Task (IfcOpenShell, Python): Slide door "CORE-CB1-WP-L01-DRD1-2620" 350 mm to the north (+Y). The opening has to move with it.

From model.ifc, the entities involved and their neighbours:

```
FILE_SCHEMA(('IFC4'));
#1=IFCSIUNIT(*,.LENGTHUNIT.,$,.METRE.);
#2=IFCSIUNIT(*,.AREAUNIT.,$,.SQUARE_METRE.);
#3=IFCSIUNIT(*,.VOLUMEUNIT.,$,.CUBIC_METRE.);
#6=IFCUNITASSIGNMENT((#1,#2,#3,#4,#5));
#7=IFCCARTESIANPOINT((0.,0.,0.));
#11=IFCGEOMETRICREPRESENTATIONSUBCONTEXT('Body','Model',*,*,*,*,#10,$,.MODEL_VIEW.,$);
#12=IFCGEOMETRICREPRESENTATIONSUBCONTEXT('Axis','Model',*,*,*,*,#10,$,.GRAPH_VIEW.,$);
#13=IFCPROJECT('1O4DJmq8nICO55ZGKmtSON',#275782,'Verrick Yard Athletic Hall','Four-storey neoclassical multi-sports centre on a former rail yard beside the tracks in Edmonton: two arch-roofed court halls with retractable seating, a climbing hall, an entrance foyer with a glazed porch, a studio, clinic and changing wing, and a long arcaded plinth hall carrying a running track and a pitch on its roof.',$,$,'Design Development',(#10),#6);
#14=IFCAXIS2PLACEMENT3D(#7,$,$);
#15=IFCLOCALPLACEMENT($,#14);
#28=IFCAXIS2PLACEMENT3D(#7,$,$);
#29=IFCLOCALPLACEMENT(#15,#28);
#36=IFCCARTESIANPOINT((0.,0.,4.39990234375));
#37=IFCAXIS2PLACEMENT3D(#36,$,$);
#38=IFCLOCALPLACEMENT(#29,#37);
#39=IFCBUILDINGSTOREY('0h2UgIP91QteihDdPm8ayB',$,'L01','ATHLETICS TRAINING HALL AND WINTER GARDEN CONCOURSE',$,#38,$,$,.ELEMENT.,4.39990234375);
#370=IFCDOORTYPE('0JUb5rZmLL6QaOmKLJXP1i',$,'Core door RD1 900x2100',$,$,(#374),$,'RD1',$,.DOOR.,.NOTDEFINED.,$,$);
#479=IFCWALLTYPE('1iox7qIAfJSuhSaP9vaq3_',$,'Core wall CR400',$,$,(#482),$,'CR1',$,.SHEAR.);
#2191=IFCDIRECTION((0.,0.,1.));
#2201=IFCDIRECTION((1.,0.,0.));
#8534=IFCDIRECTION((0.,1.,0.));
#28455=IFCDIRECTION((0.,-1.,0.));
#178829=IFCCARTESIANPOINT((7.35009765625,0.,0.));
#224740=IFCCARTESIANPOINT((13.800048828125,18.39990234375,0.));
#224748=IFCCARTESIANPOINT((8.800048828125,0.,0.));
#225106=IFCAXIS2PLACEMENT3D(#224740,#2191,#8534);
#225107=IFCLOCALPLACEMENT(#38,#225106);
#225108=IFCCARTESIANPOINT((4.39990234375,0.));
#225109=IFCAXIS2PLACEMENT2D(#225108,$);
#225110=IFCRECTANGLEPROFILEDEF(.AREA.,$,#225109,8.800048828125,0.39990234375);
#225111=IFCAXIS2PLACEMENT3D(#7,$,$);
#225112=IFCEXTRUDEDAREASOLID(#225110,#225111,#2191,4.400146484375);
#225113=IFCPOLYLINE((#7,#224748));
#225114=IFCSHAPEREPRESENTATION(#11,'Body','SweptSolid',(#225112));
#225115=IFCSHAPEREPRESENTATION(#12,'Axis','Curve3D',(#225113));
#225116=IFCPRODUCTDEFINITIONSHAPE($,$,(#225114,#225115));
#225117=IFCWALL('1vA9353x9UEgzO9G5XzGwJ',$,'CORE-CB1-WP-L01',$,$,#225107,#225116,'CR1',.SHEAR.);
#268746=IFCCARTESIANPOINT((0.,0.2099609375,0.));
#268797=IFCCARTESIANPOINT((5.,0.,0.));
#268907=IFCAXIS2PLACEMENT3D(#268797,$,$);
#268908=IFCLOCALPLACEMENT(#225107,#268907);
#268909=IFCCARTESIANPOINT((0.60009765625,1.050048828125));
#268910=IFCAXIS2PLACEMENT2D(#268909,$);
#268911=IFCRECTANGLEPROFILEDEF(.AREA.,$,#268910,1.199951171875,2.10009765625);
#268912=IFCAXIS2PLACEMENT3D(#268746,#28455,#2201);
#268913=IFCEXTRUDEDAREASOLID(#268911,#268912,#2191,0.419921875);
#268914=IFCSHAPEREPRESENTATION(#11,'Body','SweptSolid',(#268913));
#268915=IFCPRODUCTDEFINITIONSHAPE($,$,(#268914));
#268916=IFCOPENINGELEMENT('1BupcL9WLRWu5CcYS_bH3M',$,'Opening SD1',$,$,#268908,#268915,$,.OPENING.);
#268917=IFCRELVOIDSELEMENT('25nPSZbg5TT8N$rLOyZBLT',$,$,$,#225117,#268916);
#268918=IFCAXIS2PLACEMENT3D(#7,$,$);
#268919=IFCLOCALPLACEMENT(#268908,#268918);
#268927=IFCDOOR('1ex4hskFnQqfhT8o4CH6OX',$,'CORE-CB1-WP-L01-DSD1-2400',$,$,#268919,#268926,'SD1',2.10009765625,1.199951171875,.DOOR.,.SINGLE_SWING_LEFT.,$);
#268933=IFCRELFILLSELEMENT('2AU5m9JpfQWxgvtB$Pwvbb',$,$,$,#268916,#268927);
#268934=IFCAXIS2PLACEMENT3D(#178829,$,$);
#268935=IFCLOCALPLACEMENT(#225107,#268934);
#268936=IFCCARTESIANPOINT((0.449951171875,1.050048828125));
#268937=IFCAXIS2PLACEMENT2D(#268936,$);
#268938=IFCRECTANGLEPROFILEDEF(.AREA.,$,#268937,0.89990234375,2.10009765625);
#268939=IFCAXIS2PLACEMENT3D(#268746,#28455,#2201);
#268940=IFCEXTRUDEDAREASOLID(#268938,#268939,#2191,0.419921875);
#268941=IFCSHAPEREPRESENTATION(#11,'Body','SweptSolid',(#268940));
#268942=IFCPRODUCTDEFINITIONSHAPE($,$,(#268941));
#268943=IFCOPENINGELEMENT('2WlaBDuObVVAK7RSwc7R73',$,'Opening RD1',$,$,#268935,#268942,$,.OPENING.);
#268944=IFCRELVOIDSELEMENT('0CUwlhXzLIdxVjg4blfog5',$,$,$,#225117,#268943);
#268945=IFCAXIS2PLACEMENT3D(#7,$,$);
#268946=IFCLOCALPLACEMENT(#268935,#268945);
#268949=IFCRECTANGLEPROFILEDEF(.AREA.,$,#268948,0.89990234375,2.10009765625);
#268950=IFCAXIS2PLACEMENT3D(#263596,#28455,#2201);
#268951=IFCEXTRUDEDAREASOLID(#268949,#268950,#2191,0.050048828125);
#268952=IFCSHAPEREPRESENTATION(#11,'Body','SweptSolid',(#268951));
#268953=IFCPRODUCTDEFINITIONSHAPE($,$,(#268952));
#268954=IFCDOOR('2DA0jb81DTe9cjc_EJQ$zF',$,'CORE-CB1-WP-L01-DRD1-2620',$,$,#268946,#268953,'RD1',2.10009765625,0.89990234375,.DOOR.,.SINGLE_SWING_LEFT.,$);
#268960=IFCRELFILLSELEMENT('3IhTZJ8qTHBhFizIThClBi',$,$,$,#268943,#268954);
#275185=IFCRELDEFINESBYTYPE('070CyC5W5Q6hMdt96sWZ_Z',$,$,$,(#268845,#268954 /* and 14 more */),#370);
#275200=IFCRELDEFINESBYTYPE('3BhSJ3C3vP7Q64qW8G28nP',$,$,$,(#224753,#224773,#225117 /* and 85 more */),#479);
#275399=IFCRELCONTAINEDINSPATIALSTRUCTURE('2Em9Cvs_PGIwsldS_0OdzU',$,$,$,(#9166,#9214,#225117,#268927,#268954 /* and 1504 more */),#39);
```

```python
import ifcopenshell
import ifcopenshell.api.geometry
import ifcopenshell.util.placement

model = ifcopenshell.open("model.ifc")

door = model.by_guid("2DA0jb81DTe9cjc_EJQ$zF")
opening = door.FillsVoids[0].RelatingOpeningElement
wall = opening.VoidsElements[0].RelatingBuildingElement

wall_matrix = ifcopenshell.util.placement.get_local_placement(wall.ObjectPlacement)
shift = wall_matrix[:3, 0] * 0.35
before = ifcopenshell.util.placement.get_local_placement(door.ObjectPlacement)[:3, 3].copy()

# The door is placed relative to its opening, so it follows when the opening moves.
matrix = ifcopenshell.util.placement.get_local_placement(opening.ObjectPlacement)
matrix[:3, 3] += shift
ifcopenshell.api.geometry.edit_object_placement(
    model, product=opening, matrix=matrix, is_si=False, should_transform_children=True
)

after = ifcopenshell.util.placement.get_local_placement(door.ObjectPlacement)[:3, 3]
print("door moved by", (after - before).round(3) + 0.0)

model.write("model_v2.ifc")
```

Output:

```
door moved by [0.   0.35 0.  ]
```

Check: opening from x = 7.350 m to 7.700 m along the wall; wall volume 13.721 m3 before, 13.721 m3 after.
